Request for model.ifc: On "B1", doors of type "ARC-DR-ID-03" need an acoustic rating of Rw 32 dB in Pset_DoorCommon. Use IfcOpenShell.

First a look at what the model holds.

```python
import ifcopenshell
import ifcopenshell.util.element

model = ifcopenshell.open("model.ifc")
print(model.schema)
storey = next(s for s in model.by_type("IfcBuildingStorey") if s.Name == "B1")
doors = [e for e in ifcopenshell.util.element.get_decomposition(storey) if e.is_a("IfcDoor")]
seen = {}
for e in doors:
    element_type = ifcopenshell.util.element.get_type(e)
    key = (element_type.Name if element_type != e and element_type else None, ifcopenshell.util.element.get_pset(e, "Pset_DoorCommon", "AcousticRating"))
    seen[key] = seen.get(key, 0) + 1
for (name, value), count in sorted(seen.items(), key=str):
    print(count, "x", name, "|", value)
```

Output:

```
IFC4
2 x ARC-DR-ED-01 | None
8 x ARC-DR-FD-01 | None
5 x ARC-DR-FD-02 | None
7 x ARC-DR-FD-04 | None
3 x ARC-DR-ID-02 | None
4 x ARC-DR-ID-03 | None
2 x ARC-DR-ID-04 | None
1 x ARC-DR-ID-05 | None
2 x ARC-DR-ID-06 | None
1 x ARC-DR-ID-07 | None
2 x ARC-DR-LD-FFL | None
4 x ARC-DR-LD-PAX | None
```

```python
import ifcopenshell
import ifcopenshell.api.pset
import ifcopenshell.util.element

model = ifcopenshell.open("model.ifc")

storey = next(s for s in model.by_type("IfcBuildingStorey") if s.Name == "B1")
doors = [e for e in ifcopenshell.util.element.get_decomposition(storey) if e.is_a("IfcDoor")]

count = 0
for e in doors:
    element_type = ifcopenshell.util.element.get_type(e)
    if element_type in (None, e) or element_type.Name != "ARC-DR-ID-03":
        continue
    # add_pset returns the element's existing set when there is one.
    pset = ifcopenshell.api.pset.add_pset(model, product=e, name="Pset_DoorCommon")
    ifcopenshell.api.pset.edit_pset(model, pset=pset, properties={"AcousticRating": "Rw 32 dB"})
    count += 1

print(count, "doors updated")

model.write("model_edited.ifc")
```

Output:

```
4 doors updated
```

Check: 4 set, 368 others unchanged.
